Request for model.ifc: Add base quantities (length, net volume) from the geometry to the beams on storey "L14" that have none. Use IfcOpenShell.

First a look at what the model holds.

```python
import ifcopenshell
import ifcopenshell.util.element
import ifcopenshell.util.unit

model = ifcopenshell.open("model.ifc")
print(model.schema)
for unit_type in ("LENGTHUNIT", "AREAUNIT", "VOLUMEUNIT"):
    print(unit_type, ifcopenshell.util.unit.calculate_unit_scale(model, unit_type))
storey = next(s for s in model.by_type("IfcBuildingStorey") if s.Name == "L14")
beams = [e for e in ifcopenshell.util.element.get_decomposition(storey) if e.is_a("IfcBeam")]
for e in sorted(beams, key=lambda e: e.id()):
    print(e.id(), e.is_a(), e.Name, list(ifcopenshell.util.element.get_psets(e, qtos_only=True)), sep=" | ")
```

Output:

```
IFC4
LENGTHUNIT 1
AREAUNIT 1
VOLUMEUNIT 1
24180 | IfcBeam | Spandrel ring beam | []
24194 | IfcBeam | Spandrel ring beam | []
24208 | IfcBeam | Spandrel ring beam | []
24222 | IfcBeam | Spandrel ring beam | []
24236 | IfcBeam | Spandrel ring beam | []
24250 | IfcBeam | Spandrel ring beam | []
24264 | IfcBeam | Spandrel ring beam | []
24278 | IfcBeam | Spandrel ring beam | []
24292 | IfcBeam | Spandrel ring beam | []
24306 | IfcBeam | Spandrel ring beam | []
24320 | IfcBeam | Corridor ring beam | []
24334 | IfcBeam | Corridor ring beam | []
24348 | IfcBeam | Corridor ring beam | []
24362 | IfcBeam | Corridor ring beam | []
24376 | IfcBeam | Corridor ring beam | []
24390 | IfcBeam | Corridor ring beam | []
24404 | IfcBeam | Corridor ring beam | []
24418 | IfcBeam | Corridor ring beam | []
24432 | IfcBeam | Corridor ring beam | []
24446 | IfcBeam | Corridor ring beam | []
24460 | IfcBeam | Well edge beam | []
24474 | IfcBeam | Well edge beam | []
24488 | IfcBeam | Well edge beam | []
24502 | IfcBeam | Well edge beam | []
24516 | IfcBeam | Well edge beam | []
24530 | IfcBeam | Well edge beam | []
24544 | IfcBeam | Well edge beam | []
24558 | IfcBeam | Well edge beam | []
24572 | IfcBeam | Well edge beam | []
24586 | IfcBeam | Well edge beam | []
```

```python
import ifcopenshell
import ifcopenshell.api.pset
import ifcopenshell.geom
import ifcopenshell.util.element
import ifcopenshell.util.shape
import ifcopenshell.util.unit

model = ifcopenshell.open("model.ifc")
unit_scale = ifcopenshell.util.unit.calculate_unit_scale(model)
volume_scale = ifcopenshell.util.unit.calculate_unit_scale(model, "VOLUMEUNIT")
settings = ifcopenshell.geom.settings()

storey = next(s for s in model.by_type("IfcBuildingStorey") if s.Name == "L14")
beams = [e for e in ifcopenshell.util.element.get_decomposition(storey) if e.is_a("IfcBeam")]

for e in sorted(beams, key=lambda e: e.id()):
    if ifcopenshell.util.element.get_psets(e, qtos_only=True, should_inherit=False):
        continue
    # Geometry comes back in metres, in the element's own axes.
    shape = ifcopenshell.geom.create_shape(settings, e)
    values = {
        "Length": ifcopenshell.util.shape.get_max_xyz(shape.geometry) / unit_scale,
        "NetVolume": ifcopenshell.util.shape.get_volume(shape.geometry) / volume_scale,
    }
    qto = ifcopenshell.api.pset.add_qto(model, product=e, name="Qto_BeamBaseQuantities")
    ifcopenshell.api.pset.edit_qto(model, qto=qto, properties=values)
    print(e.id(), {k: round(v, 3) for k, v in values.items()})

model.write("model_rev.ifc")
```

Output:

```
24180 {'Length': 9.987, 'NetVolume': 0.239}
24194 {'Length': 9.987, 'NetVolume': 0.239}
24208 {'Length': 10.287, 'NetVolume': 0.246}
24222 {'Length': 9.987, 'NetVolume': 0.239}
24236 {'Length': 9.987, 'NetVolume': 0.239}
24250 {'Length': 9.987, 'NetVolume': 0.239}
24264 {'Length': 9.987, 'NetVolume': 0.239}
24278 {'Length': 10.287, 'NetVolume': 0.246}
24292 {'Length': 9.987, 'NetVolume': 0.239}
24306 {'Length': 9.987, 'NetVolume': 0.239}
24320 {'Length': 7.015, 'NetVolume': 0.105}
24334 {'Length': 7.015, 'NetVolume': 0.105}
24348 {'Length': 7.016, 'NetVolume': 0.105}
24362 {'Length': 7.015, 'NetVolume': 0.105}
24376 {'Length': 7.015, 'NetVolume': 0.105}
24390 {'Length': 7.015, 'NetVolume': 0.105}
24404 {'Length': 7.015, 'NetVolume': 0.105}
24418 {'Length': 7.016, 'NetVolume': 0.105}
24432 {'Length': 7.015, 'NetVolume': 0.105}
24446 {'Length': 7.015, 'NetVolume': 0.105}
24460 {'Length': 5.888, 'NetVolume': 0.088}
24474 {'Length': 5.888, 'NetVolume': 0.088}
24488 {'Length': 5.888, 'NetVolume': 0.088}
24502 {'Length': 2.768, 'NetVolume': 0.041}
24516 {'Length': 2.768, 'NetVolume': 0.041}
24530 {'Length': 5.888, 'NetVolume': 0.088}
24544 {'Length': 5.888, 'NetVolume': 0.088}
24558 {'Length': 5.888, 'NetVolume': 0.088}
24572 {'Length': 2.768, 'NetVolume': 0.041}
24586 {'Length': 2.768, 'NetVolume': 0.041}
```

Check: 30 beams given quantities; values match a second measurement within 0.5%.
